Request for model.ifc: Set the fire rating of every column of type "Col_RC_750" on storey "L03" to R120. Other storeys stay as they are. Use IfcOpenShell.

First a look at what the model holds.

```python
import ifcopenshell
import ifcopenshell.util.element

model = ifcopenshell.open("model.ifc")
print(model.schema)
storey = next(s for s in model.by_type("IfcBuildingStorey") if s.Name == "L03")
columns = [e for e in ifcopenshell.util.element.get_decomposition(storey) if e.is_a("IfcColumn")]
seen = {}
for e in columns:
    element_type = ifcopenshell.util.element.get_type(e)
    key = (element_type.Name if element_type != e and element_type else None, ifcopenshell.util.element.get_pset(e, "Pset_ColumnCommon", "FireRating"))
    seen[key] = seen.get(key, 0) + 1
for (name, value), count in sorted(seen.items(), key=str):
    print(count, "x", name, "|", value)
```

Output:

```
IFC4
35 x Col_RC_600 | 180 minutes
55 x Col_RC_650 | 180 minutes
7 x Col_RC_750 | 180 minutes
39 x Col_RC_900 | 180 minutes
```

```python
import ifcopenshell
import ifcopenshell.api.pset
import ifcopenshell.util.element

model = ifcopenshell.open("model.ifc")

storey = next(s for s in model.by_type("IfcBuildingStorey") if s.Name == "L03")
columns = [e for e in ifcopenshell.util.element.get_decomposition(storey) if e.is_a("IfcColumn")]

count = 0
for e in columns:
    element_type = ifcopenshell.util.element.get_type(e)
    if element_type in (None, e) or element_type.Name != "Col_RC_750":
        continue
    # add_pset returns the element's existing set when there is one.
    pset = ifcopenshell.api.pset.add_pset(model, product=e, name="Pset_ColumnCommon")
    ifcopenshell.api.pset.edit_pset(model, pset=pset, properties={"FireRating": "R120"})
    count += 1

print(count, "columns updated")

model.write("model_rev.ifc")
```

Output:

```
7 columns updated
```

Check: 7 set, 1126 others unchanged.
